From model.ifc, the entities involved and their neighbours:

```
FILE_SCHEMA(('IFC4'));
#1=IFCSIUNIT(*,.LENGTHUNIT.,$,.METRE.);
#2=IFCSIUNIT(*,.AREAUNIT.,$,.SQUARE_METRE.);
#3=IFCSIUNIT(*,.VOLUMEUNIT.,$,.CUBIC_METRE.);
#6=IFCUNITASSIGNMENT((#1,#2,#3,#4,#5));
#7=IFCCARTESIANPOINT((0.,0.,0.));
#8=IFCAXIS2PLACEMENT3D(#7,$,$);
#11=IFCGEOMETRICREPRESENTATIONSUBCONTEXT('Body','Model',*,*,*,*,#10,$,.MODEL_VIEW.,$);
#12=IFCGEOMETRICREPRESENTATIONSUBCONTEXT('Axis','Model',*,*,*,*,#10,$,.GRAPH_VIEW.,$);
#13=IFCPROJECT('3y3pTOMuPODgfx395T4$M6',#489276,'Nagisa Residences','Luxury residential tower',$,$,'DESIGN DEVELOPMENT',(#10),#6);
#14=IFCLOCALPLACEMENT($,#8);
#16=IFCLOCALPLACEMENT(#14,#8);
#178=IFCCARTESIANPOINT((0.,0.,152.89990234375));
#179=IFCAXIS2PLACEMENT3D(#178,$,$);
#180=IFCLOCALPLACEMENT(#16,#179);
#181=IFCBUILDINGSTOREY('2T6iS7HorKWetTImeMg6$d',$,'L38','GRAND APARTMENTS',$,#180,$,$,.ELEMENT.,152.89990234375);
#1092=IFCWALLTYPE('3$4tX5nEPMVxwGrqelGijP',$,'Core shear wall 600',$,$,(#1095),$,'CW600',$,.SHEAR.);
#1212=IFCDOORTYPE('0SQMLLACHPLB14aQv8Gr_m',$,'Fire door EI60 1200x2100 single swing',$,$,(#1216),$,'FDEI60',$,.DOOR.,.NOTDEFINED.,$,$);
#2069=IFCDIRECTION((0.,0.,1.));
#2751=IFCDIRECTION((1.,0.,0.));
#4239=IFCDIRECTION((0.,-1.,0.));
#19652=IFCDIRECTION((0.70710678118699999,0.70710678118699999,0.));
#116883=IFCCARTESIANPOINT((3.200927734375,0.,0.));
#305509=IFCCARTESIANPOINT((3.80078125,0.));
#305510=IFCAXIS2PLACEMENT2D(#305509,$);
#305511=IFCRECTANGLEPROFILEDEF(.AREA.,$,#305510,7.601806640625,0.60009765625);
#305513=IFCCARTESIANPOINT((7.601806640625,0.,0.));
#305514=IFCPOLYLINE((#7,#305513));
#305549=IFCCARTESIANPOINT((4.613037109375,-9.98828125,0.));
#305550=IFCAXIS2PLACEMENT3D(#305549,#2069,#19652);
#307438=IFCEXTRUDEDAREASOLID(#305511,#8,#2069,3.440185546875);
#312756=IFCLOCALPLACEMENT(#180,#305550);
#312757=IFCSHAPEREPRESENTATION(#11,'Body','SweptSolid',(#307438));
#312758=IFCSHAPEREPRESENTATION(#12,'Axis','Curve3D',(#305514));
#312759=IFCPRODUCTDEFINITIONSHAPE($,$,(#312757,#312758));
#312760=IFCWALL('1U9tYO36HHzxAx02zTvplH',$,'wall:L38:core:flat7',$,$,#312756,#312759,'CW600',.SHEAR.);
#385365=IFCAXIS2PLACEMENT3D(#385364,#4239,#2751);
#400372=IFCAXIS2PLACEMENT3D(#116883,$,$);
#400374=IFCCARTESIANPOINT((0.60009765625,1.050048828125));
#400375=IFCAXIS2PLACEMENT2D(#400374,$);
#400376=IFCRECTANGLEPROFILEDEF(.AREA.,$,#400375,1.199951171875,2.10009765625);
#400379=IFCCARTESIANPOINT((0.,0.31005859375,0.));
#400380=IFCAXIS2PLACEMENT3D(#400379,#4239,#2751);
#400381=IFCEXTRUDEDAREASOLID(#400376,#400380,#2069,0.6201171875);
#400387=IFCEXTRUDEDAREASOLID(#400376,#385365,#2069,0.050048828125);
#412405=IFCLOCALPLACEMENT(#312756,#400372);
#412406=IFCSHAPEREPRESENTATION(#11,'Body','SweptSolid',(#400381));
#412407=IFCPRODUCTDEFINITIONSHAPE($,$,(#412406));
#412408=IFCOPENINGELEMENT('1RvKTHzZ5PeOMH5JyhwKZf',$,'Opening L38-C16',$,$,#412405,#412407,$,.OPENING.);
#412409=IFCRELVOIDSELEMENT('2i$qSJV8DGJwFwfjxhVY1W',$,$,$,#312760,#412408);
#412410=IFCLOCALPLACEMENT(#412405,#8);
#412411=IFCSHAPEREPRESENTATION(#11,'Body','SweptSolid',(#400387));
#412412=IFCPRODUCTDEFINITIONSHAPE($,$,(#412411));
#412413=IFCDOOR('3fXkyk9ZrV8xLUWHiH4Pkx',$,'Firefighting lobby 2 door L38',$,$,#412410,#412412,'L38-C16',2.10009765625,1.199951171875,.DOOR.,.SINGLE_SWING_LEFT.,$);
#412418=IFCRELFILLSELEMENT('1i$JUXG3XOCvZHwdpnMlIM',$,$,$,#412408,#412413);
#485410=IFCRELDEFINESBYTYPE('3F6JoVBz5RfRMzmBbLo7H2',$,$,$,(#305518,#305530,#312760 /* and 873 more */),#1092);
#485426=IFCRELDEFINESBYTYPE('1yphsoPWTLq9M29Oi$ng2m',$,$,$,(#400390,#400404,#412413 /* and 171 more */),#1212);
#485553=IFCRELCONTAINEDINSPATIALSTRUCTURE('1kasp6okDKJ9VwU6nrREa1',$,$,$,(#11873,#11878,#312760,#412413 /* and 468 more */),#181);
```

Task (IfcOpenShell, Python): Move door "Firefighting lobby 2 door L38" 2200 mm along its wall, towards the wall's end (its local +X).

```python
import ifcopenshell
import ifcopenshell.api.geometry
import ifcopenshell.util.placement

model = ifcopenshell.open("model.ifc")

door = model.by_guid("3fXkyk9ZrV8xLUWHiH4Pkx")
opening = door.FillsVoids[0].RelatingOpeningElement
wall = opening.VoidsElements[0].RelatingBuildingElement

wall_matrix = ifcopenshell.util.placement.get_local_placement(wall.ObjectPlacement)
shift = wall_matrix[:3, 0] * 2.2
before = ifcopenshell.util.placement.get_local_placement(door.ObjectPlacement)[:3, 3].copy()

# The door is placed relative to its opening, so it follows when the opening moves.
matrix = ifcopenshell.util.placement.get_local_placement(opening.ObjectPlacement)
matrix[:3, 3] += shift
ifcopenshell.api.geometry.edit_object_placement(
    model, product=opening, matrix=matrix, is_si=False, should_transform_children=True
)

after = ifcopenshell.util.placement.get_local_placement(door.ObjectPlacement)[:3, 3]
print("door moved by", (after - before).round(3) + 0.0)

model.write("model_edited.ifc")
```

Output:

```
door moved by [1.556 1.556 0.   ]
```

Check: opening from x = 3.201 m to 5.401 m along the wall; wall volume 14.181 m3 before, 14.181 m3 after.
